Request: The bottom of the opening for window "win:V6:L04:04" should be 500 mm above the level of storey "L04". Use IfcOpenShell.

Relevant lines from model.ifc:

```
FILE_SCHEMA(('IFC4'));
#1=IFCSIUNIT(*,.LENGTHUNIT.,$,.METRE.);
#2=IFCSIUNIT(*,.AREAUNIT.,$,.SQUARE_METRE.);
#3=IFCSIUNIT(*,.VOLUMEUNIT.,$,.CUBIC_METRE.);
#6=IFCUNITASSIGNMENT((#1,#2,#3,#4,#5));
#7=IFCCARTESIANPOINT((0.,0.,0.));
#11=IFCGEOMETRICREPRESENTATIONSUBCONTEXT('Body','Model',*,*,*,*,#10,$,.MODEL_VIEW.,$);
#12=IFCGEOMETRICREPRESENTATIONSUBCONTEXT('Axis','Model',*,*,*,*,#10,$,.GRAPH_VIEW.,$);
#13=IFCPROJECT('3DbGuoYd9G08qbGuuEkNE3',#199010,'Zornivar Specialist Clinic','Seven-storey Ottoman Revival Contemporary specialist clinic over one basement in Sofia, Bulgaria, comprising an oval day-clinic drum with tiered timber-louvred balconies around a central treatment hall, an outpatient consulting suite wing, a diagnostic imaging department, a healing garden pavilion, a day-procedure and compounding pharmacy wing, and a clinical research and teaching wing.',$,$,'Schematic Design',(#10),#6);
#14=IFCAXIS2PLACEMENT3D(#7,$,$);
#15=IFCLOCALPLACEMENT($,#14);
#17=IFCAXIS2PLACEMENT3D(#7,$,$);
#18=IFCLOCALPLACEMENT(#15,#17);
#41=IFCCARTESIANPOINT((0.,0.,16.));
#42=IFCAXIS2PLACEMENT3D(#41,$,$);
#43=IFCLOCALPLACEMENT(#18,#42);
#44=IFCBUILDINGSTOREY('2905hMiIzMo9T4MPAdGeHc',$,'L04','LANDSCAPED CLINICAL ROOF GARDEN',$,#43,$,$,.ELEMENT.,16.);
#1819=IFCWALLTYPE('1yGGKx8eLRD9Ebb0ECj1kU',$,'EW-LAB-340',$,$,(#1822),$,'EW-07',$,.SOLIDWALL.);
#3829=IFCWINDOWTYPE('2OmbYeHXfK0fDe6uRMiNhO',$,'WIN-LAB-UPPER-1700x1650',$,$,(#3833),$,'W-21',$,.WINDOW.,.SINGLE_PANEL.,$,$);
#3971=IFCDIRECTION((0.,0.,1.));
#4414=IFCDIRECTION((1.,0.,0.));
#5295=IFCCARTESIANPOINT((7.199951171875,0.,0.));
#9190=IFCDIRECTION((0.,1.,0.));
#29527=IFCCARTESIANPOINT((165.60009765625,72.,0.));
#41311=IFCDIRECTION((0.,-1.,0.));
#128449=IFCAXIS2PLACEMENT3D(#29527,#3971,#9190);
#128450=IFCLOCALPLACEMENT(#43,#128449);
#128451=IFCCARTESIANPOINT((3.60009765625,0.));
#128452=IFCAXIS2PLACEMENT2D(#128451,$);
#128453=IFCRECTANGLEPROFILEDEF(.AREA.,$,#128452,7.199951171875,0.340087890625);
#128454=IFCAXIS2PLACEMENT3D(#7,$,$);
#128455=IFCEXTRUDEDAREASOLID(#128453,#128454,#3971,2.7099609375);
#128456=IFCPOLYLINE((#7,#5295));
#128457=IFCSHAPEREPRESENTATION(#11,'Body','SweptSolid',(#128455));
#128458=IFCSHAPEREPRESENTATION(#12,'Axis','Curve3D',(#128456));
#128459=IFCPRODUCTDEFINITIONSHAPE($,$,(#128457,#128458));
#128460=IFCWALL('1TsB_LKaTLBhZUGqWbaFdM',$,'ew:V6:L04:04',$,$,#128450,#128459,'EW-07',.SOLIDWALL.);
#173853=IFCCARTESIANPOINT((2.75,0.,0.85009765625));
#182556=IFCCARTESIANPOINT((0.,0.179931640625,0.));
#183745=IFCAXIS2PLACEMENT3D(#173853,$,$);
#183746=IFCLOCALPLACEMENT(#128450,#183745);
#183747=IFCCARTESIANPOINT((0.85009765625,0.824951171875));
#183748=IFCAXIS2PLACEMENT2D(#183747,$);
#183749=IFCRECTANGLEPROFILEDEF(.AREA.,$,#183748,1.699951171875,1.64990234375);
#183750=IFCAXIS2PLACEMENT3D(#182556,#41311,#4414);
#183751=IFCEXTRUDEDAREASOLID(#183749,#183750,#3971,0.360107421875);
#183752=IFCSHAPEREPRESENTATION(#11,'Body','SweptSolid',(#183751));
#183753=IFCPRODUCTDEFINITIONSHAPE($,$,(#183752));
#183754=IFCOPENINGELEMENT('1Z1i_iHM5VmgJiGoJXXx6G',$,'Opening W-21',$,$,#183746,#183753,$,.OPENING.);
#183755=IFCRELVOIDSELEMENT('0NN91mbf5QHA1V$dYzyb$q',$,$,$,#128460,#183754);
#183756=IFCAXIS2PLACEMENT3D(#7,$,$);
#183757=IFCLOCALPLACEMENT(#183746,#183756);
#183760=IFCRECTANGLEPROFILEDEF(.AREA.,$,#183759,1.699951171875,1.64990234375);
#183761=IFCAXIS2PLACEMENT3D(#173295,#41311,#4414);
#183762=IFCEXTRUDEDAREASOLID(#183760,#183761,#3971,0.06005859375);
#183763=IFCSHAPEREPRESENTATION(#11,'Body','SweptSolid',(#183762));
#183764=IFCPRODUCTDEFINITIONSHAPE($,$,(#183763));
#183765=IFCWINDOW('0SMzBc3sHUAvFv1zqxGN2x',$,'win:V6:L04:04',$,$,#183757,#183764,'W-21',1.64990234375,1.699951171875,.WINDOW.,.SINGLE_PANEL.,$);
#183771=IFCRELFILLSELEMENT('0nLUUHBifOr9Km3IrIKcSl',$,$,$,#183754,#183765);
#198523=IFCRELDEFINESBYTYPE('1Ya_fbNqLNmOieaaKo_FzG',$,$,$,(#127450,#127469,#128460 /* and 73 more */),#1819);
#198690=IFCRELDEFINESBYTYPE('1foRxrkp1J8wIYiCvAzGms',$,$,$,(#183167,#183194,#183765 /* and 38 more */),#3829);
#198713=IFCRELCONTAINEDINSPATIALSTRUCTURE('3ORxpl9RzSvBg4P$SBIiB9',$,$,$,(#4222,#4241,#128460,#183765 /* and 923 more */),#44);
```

```python
import numpy as np
import ifcopenshell
import ifcopenshell.api.geometry
import ifcopenshell.geom
import ifcopenshell.util.element
import ifcopenshell.util.placement
import ifcopenshell.util.shape
import ifcopenshell.util.unit

model = ifcopenshell.open("model.ifc")
unit_scale = ifcopenshell.util.unit.calculate_unit_scale(model)

window = model.by_guid("0SMzBc3sHUAvFv1zqxGN2x")
opening = window.FillsVoids[0].RelatingOpeningElement
storey = ifcopenshell.util.element.get_container(window, ifc_class="IfcBuildingStorey")
level = ifcopenshell.util.placement.get_local_placement(storey.ObjectPlacement)[2, 3]

# The opening's origin need not be at the sill, so measure its lowest point.
shape = ifcopenshell.geom.create_shape(ifcopenshell.geom.settings(), opening)
bottom = ifcopenshell.util.shape.get_shape_bottom_elevation(shape, shape.geometry) / unit_scale
dz = level + 0.5 / unit_scale - bottom

shift = np.array([0.0, 0.0, dz])
# The window is placed relative to its opening, so it follows when the opening moves.
matrix = ifcopenshell.util.placement.get_local_placement(opening.ObjectPlacement)
matrix[:3, 3] += shift
ifcopenshell.api.geometry.edit_object_placement(
    model, product=opening, matrix=matrix, is_si=False, should_transform_children=True
)

print(f"moved by {dz * unit_scale:+.3f} m")

model.write("model_v2.ifc")
```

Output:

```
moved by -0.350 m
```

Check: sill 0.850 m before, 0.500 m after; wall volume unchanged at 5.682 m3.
